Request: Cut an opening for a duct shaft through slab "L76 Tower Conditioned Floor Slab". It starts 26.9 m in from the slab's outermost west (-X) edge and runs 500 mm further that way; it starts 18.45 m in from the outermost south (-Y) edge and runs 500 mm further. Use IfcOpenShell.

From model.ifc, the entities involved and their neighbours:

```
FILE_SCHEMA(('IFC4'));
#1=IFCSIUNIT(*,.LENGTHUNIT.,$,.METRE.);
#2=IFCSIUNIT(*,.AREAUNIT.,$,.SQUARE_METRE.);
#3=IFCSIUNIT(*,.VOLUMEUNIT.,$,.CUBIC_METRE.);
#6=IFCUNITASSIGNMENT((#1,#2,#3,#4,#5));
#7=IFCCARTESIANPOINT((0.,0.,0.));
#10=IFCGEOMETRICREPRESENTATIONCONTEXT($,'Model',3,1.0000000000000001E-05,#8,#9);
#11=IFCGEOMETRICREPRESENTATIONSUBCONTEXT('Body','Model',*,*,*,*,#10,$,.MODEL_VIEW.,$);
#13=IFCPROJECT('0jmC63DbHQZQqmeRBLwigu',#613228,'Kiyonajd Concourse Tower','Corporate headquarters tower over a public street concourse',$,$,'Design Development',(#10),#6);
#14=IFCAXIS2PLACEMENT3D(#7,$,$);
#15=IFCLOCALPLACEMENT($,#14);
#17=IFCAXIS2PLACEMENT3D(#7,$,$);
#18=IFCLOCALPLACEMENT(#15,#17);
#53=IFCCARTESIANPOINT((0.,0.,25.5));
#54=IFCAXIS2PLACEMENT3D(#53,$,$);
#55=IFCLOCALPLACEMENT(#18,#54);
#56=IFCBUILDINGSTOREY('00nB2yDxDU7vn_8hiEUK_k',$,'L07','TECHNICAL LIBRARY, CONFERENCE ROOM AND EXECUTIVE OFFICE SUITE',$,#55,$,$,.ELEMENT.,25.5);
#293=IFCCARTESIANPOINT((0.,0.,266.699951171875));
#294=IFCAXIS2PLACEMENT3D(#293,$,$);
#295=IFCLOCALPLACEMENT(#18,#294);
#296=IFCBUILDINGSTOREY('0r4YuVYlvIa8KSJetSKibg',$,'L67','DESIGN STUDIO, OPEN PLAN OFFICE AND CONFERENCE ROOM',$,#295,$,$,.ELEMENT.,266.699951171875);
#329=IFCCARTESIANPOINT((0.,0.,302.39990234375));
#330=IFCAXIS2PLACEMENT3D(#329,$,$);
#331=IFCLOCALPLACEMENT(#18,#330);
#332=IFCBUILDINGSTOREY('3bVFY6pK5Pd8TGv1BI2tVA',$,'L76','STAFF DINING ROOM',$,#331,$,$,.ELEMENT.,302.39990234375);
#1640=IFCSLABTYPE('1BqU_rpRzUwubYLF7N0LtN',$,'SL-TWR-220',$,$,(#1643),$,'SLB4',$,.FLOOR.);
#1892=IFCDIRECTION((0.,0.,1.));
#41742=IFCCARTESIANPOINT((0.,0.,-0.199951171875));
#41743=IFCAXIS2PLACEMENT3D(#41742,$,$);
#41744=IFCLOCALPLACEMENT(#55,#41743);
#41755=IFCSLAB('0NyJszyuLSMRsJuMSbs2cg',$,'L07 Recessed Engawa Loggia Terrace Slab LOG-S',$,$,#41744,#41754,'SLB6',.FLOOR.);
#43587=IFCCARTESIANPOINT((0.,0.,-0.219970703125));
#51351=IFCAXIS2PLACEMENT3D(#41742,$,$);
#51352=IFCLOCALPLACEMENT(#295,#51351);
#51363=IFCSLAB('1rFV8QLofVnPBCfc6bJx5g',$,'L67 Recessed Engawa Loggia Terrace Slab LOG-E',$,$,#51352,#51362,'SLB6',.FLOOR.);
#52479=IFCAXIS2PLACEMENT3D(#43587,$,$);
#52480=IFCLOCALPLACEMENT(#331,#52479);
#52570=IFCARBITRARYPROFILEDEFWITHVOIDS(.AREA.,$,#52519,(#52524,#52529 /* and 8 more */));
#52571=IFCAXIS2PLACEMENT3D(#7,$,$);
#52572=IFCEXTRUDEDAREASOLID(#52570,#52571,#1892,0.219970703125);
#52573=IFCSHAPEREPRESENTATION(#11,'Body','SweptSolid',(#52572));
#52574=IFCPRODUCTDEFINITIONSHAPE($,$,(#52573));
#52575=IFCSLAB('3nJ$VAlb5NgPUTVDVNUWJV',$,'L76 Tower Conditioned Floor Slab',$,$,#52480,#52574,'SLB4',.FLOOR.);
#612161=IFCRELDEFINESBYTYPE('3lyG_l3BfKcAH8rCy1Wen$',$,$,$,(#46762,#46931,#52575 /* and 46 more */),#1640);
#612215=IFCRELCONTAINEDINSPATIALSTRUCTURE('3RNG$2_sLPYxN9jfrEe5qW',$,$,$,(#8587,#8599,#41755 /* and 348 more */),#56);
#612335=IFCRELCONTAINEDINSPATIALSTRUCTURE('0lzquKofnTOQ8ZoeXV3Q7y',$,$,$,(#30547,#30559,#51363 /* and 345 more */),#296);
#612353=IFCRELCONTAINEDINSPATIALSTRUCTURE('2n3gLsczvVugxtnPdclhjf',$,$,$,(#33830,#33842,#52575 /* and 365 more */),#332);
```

```python
import numpy as np
import ifcopenshell
import ifcopenshell.api.feature
import ifcopenshell.api.geometry
import ifcopenshell.api.root
import ifcopenshell.geom
import ifcopenshell.util.placement
import ifcopenshell.util.representation
import ifcopenshell.util.shape
import ifcopenshell.util.unit

model = ifcopenshell.open("model.ifc")
unit_scale = ifcopenshell.util.unit.calculate_unit_scale(model)
settings = ifcopenshell.geom.settings()


def volume(element):
    """Net volume in cubic metres, openings subtracted."""
    shape = ifcopenshell.geom.create_shape(settings, element)
    return ifcopenshell.util.shape.get_volume(shape.geometry)


slab = model.by_guid("3nJ$VAlb5NgPUTVDVNUWJV")
before = volume(slab)

# Extent in the slab's own axes, in metres. The edges named are its -X and -Y sides.
slab_shape = ifcopenshell.geom.create_shape(settings, slab)
vertices = ifcopenshell.util.shape.get_vertices(slab_shape.geometry)
x_min, y_min, bottom = vertices.min(axis=0)
top = vertices[:, 2].max()

opening = ifcopenshell.api.root.create_entity(model, ifc_class="IfcOpeningElement", name="Duct shaft opening", predefined_type="OPENING")
context = ifcopenshell.util.representation.get_context(model, "Model", "Body", "MODEL_VIEW")
width, depth = 0.5, 0.5
outline = [(0.0, 0.0), (width, 0.0), (width, depth), (0.0, depth), (0.0, 0.0)]
# Overshoot both faces by 50 mm so the cut is clean.
shape = ifcopenshell.api.geometry.add_slab_representation(
    model, context=context, depth=top - bottom + 0.1, polyline=outline
)
ifcopenshell.api.geometry.assign_representation(model, product=opening, representation=shape)

matrix = ifcopenshell.util.placement.get_local_placement(slab.ObjectPlacement)
matrix[:, 3] = matrix @ np.append(np.array([x_min + 26.9, y_min + 18.45, bottom - 0.05]) / unit_scale, 1.0)
ifcopenshell.api.geometry.edit_object_placement(model, product=opening, matrix=matrix, is_si=False)
ifcopenshell.api.feature.add_feature(model, feature=opening, element=slab)

after = volume(slab)

print(f"slab volume {before:.3f} -> {after:.3f} m3")

model.write("model_updated.ifc")
```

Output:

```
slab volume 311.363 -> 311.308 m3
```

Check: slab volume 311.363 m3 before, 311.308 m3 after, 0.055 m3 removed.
